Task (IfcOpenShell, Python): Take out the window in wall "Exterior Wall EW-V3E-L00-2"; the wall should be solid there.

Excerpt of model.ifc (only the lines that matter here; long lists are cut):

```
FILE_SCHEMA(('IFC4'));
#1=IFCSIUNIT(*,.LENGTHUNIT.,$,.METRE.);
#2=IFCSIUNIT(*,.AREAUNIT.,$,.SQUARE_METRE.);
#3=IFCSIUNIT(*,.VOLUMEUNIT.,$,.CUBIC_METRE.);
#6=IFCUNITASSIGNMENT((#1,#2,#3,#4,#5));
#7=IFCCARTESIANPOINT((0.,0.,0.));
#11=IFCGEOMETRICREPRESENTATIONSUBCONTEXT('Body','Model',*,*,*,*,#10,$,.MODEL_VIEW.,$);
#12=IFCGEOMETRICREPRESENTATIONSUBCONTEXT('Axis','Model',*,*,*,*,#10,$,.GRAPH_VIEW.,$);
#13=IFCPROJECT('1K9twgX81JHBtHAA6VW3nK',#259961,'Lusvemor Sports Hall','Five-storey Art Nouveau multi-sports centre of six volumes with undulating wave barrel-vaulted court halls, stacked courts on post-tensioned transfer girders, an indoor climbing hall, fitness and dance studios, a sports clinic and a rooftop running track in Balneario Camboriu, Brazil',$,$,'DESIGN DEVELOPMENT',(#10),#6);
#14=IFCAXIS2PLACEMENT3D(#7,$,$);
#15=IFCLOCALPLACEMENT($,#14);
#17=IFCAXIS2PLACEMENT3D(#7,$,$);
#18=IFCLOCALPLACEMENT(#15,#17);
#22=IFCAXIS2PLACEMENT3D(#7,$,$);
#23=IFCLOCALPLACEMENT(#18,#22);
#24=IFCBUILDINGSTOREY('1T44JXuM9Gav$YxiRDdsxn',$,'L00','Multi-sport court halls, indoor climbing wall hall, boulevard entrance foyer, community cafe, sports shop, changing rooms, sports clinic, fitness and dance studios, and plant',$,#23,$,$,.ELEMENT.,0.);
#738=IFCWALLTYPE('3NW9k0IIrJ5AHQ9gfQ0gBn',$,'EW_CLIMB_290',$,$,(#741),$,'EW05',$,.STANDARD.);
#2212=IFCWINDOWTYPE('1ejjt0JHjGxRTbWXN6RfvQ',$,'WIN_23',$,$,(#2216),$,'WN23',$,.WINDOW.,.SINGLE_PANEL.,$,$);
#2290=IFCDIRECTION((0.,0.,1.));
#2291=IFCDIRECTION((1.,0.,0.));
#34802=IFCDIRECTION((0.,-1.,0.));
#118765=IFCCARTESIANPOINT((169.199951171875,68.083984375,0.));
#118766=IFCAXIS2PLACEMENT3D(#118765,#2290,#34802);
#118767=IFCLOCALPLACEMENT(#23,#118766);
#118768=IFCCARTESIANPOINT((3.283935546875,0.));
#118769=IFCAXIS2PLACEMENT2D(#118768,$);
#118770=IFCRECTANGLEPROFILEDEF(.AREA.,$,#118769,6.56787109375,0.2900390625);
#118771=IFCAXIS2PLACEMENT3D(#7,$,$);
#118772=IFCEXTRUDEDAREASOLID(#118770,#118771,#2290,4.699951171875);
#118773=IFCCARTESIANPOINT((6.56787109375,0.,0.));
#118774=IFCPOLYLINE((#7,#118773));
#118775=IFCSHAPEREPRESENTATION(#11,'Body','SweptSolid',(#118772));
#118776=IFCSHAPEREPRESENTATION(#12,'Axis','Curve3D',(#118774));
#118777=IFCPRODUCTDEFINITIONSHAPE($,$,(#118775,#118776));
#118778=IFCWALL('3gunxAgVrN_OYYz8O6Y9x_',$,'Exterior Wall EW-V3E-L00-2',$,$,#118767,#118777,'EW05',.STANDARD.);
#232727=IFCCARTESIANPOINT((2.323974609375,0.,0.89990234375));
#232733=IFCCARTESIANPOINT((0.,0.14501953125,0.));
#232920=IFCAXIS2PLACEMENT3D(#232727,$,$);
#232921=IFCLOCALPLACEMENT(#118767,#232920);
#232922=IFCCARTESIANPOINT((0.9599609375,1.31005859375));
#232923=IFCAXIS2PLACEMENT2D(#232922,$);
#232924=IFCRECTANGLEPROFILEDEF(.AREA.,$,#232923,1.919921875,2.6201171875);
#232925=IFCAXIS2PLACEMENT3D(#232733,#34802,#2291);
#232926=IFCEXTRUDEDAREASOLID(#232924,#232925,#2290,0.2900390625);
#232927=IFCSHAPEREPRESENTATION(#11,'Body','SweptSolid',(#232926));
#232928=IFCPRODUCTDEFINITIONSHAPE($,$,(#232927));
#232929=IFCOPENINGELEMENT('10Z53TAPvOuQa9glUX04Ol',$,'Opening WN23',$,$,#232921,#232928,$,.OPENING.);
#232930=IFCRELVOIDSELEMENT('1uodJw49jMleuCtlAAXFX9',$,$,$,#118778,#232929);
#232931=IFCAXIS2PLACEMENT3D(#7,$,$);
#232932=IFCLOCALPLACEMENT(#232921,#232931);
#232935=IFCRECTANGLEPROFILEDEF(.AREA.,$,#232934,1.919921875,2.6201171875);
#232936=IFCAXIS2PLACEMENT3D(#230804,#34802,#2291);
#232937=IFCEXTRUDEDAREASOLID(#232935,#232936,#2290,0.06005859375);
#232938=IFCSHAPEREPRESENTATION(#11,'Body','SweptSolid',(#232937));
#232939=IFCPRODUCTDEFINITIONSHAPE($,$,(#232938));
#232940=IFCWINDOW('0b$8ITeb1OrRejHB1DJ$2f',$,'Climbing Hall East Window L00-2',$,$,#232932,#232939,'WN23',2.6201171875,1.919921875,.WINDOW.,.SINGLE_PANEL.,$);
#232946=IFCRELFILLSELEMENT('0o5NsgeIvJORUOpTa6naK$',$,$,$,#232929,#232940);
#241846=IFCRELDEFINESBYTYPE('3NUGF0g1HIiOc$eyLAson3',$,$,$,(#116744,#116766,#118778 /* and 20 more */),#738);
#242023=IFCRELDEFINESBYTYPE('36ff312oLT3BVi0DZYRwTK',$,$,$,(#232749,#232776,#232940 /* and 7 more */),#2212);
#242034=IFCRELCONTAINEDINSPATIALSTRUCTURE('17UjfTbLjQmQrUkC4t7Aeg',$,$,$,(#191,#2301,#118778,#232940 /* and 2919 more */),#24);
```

```python
import ifcopenshell
import ifcopenshell.api.feature
import ifcopenshell.api.root
import ifcopenshell.geom
import ifcopenshell.util.shape

model = ifcopenshell.open("model.ifc")
settings = ifcopenshell.geom.settings()


def volume(element):
    """Net volume in cubic metres, openings subtracted."""
    shape = ifcopenshell.geom.create_shape(settings, element)
    return ifcopenshell.util.shape.get_volume(shape.geometry)


window = model.by_guid("0b$8ITeb1OrRejHB1DJ$2f")
opening = window.FillsVoids[0].RelatingOpeningElement
wall = opening.VoidsElements[0].RelatingBuildingElement
before = volume(wall)

ifcopenshell.api.root.remove_product(model, product=window)
ifcopenshell.api.feature.remove_feature(model, feature=opening)

after = volume(wall)

print(f"wall volume {before:.3f} -> {after:.3f} m3")

model.write("model_updated.ifc")
```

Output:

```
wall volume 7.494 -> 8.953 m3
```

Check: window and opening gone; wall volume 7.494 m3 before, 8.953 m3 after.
